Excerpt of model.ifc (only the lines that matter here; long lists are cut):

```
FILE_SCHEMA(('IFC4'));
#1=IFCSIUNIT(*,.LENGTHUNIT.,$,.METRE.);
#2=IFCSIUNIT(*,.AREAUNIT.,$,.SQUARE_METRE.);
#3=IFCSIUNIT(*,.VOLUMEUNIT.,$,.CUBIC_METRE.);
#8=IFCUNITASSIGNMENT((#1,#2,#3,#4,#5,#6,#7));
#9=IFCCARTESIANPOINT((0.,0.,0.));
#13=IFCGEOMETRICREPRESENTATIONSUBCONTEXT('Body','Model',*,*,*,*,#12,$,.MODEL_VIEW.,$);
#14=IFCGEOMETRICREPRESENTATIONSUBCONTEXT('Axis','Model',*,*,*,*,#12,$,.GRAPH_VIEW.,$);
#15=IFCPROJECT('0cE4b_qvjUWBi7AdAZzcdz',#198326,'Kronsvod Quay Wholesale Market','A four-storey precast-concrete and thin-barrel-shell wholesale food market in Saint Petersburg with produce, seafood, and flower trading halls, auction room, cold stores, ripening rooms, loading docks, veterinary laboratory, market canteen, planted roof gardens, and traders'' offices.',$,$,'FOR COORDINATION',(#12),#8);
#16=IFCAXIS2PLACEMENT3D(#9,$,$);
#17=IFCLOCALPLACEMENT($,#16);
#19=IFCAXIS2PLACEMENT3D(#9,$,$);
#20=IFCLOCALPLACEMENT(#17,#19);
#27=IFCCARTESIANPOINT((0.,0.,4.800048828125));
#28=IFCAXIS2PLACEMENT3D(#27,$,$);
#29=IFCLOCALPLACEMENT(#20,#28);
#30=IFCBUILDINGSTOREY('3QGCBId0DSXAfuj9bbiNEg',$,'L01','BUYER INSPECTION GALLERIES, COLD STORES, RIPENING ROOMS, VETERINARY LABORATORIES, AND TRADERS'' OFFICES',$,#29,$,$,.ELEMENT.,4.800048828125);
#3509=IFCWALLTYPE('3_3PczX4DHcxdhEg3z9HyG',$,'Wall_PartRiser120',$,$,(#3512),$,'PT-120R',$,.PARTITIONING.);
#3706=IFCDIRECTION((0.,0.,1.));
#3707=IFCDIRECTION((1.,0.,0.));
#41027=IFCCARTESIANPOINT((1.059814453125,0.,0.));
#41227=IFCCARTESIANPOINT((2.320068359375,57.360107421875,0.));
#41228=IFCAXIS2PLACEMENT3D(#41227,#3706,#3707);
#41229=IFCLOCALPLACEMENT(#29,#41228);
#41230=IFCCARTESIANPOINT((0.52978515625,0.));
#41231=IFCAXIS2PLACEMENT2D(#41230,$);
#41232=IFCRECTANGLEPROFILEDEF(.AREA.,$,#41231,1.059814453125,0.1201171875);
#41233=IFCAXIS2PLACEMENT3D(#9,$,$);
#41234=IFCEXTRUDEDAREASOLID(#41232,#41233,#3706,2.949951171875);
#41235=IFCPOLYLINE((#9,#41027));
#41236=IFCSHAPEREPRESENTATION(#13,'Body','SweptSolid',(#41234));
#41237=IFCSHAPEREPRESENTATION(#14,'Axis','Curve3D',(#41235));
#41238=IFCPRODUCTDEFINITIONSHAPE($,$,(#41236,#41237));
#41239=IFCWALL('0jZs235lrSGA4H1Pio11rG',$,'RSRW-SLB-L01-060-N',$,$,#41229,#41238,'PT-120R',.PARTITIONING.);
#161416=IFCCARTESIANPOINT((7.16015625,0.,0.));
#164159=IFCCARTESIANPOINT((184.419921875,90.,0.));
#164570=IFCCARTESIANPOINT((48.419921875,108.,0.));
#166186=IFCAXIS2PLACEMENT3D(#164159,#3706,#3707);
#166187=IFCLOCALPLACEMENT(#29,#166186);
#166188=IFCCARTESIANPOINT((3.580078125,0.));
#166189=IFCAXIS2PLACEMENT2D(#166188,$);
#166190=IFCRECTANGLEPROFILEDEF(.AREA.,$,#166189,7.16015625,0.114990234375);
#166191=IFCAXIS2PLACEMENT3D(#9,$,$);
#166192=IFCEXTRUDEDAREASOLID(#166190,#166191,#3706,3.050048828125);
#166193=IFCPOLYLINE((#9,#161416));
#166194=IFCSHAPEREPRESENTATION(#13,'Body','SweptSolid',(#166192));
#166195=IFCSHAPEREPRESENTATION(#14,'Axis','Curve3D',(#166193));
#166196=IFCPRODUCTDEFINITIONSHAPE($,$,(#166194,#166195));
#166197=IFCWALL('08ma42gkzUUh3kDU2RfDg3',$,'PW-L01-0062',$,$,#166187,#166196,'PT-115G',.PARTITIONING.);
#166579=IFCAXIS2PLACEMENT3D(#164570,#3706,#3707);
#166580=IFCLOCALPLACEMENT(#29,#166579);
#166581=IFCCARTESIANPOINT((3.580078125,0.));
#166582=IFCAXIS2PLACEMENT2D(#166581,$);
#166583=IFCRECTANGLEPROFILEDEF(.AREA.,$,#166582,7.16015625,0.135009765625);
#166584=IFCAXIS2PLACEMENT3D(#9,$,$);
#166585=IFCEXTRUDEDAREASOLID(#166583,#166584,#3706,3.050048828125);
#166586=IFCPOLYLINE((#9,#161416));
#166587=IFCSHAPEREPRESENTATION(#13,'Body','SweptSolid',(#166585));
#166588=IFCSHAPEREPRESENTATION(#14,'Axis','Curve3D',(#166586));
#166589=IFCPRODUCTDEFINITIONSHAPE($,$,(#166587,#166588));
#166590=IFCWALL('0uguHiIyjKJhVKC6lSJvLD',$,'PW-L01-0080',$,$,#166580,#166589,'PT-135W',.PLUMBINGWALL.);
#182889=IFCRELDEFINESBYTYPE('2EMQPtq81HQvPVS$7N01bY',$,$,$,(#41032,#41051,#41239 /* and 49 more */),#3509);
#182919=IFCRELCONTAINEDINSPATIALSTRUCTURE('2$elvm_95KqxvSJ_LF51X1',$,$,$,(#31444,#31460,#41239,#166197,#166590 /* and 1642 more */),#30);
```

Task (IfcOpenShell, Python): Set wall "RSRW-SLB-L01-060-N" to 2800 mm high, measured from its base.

```python
import ifcopenshell
import ifcopenshell.geom
import ifcopenshell.util.representation
import ifcopenshell.util.shape
import ifcopenshell.util.unit

model = ifcopenshell.open("model.ifc")
unit_scale = ifcopenshell.util.unit.calculate_unit_scale(model)
settings = ifcopenshell.geom.settings()


def volume(element):
    """Net volume in cubic metres, openings subtracted."""
    shape = ifcopenshell.geom.create_shape(settings, element)
    return ifcopenshell.util.shape.get_volume(shape.geometry)


wall = model.by_id(41239)
before = volume(wall)

body = ifcopenshell.util.representation.get_representation(wall, "Model", "Body")
solid = body.Items[0]
old_height = solid.Depth
solid.Depth = 2.8 / unit_scale
after = volume(wall)

print(f"height {old_height:g} -> {solid.Depth:g}, volume {before:.3f} -> {after:.3f} m3")

model.write("model_rev.ifc")
```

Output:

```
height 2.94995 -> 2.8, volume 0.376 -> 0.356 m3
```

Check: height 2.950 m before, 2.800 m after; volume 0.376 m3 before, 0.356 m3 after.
